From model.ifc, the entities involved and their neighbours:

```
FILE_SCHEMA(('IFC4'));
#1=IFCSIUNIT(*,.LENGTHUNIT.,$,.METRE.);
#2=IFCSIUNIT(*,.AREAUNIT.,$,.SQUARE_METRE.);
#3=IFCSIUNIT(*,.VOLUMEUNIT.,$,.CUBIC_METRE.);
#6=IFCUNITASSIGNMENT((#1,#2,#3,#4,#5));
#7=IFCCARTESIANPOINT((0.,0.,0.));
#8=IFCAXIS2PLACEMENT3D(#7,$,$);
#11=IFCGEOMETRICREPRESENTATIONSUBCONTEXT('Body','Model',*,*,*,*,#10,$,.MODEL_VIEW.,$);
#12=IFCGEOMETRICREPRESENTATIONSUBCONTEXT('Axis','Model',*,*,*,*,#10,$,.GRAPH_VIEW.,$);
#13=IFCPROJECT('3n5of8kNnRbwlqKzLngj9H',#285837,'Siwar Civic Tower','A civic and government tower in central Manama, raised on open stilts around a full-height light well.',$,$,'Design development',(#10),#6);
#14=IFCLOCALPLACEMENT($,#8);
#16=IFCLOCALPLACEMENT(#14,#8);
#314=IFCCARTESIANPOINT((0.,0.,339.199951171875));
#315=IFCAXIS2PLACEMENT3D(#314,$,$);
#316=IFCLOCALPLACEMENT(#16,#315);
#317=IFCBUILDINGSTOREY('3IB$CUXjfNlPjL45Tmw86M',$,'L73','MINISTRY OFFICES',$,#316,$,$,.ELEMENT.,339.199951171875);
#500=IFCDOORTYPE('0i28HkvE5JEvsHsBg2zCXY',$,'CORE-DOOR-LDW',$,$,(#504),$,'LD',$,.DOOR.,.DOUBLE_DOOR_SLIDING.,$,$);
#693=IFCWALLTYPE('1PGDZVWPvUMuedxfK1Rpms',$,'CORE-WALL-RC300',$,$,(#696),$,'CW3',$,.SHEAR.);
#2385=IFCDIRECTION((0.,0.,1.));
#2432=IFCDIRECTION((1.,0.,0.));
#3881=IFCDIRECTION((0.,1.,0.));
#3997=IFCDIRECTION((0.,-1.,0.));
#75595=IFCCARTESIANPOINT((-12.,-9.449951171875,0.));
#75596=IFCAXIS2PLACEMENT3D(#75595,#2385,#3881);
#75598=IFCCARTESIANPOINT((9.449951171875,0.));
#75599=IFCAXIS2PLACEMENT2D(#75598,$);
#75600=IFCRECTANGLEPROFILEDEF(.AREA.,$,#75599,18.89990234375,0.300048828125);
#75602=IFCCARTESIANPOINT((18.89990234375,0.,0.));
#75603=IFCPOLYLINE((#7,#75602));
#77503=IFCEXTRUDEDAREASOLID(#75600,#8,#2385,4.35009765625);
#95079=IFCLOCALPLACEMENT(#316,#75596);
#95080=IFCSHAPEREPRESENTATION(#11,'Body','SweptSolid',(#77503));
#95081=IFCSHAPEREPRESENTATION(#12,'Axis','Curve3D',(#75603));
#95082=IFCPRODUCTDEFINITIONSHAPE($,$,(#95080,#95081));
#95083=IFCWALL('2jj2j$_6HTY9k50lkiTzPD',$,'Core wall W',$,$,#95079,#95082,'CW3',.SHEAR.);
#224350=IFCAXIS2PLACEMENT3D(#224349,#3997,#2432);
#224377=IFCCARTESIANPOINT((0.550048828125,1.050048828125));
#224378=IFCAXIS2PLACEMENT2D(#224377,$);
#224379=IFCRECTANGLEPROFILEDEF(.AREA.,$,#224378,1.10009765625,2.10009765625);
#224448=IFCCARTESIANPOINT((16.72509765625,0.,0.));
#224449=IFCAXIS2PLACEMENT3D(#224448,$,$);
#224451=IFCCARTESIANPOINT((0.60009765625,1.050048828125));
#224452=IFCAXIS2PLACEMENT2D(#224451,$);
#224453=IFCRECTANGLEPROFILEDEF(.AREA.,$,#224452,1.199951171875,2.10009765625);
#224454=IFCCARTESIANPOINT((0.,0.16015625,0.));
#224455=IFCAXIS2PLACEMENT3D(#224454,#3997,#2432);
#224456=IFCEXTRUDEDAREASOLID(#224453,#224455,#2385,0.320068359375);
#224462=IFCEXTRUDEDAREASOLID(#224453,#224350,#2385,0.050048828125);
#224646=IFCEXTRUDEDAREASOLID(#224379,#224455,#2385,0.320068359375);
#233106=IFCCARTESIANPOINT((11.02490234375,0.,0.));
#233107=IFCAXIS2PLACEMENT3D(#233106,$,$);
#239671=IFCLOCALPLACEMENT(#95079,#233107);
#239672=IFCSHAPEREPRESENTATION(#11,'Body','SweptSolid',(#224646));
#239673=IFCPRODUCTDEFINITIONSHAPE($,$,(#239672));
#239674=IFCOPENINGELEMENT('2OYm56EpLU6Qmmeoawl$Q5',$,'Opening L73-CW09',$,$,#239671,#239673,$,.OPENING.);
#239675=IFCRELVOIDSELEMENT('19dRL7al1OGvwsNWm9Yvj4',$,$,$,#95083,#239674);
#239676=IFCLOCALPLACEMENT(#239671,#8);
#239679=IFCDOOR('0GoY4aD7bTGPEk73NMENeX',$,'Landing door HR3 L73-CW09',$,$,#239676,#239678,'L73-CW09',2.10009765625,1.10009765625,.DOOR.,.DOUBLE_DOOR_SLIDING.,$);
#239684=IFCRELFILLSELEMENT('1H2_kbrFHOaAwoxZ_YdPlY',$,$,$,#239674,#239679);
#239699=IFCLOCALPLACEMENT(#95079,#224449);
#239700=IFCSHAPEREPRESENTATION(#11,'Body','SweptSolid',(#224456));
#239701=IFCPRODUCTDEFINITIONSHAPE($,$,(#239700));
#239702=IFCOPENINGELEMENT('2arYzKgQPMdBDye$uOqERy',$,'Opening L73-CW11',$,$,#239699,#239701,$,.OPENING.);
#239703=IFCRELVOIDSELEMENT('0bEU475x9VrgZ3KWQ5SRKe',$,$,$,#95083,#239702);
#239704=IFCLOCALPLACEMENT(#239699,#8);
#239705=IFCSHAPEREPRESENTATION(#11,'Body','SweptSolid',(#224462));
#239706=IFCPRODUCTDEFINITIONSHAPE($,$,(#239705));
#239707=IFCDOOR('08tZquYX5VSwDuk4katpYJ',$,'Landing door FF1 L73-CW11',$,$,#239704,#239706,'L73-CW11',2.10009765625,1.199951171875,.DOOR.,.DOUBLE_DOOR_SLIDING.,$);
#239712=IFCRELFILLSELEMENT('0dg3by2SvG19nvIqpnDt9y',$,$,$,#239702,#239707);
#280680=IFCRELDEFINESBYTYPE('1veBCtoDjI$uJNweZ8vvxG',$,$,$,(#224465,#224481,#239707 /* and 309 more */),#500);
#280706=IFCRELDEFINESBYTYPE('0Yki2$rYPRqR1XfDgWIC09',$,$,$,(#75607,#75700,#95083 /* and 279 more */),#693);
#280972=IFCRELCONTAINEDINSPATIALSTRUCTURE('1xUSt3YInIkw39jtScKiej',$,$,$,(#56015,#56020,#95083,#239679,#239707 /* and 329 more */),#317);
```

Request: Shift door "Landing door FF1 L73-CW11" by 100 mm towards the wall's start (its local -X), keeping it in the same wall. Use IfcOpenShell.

```python
import ifcopenshell
import ifcopenshell.api.geometry
import ifcopenshell.util.placement
import ifcopenshell.util.unit

model = ifcopenshell.open("model.ifc")
unit_scale = ifcopenshell.util.unit.calculate_unit_scale(model)

door = model.by_id(239707)
opening = door.FillsVoids[0].RelatingOpeningElement
wall = opening.VoidsElements[0].RelatingBuildingElement

wall_matrix = ifcopenshell.util.placement.get_local_placement(wall.ObjectPlacement)
shift = wall_matrix[:3, 0] * -0.1 / unit_scale
before = ifcopenshell.util.placement.get_local_placement(door.ObjectPlacement)[:3, 3].copy()

# The door is placed relative to its opening, so it follows when the opening moves.
matrix = ifcopenshell.util.placement.get_local_placement(opening.ObjectPlacement)
matrix[:3, 3] += shift
ifcopenshell.api.geometry.edit_object_placement(
    model, product=opening, matrix=matrix, is_si=False, should_transform_children=True
)

after = ifcopenshell.util.placement.get_local_placement(door.ObjectPlacement)[:3, 3]
print("door moved by", (after - before).round(3) + 0.0)

model.write("model_updated.ifc")
```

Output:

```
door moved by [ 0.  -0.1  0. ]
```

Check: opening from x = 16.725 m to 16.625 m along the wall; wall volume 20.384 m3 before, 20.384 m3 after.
